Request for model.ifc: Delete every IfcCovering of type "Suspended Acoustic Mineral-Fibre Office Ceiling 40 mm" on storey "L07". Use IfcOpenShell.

First a look at what the model holds.

```python
import ifcopenshell
import ifcopenshell.util.element

model = ifcopenshell.open("model.ifc")
print(model.schema)
storey = next(s for s in model.by_type("IfcBuildingStorey") if s.Name == "L07")
coverings = [e for e in ifcopenshell.util.element.get_decomposition(storey) if e.is_a("IfcCovering")]
seen = {}
for e in coverings:
    element_type = ifcopenshell.util.element.get_type(e)
    name = element_type.Name if element_type not in (None, e) else None
    seen[name] = seen.get(name, 0) + 1
for name, count in sorted(seen.items(), key=str):
    print(count, "x", name)
```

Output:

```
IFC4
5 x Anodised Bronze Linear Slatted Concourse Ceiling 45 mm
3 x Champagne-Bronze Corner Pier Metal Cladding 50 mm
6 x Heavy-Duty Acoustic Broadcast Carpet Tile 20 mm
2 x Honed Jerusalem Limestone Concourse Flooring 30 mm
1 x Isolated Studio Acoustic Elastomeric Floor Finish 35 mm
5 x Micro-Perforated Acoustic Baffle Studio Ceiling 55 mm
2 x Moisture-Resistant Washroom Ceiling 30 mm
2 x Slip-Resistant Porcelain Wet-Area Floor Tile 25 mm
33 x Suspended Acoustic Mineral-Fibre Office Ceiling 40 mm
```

```python
import ifcopenshell
import ifcopenshell.api.root
import ifcopenshell.util.element

model = ifcopenshell.open("model.ifc")

storey = next(s for s in model.by_type("IfcBuildingStorey") if s.Name == "L07")
coverings = [e for e in ifcopenshell.util.element.get_decomposition(storey) if e.is_a("IfcCovering")]
targets = [e for e in coverings if (t := ifcopenshell.util.element.get_type(e)) not in (None, e) and t.Name == "Suspended Acoustic Mineral-Fibre Office Ceiling 40 mm"]

for e in targets:
    ifcopenshell.api.root.remove_product(model, product=e)
print(len(targets), "removed")

model.write("model_updated.ifc")
```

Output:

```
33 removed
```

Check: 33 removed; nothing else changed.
